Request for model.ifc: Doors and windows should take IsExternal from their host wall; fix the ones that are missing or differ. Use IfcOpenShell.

First a look at what the model holds.

```python
import ifcopenshell
import ifcopenshell.util.element

model = ifcopenshell.open("model.ifc")
print(model.schema)
seen = {}
for e in model.by_type("IfcDoor") + model.by_type("IfcWindow"):
    if not e.FillsVoids:
        continue
    host = e.FillsVoids[0].RelatingOpeningElement.VoidsElements[0].RelatingBuildingElement
    own = ifcopenshell.util.element.get_pset(e, f"Pset_{e.is_a()[3:].removesuffix('StandardCase')}Common", "IsExternal")
    wall = ifcopenshell.util.element.get_pset(host, "Pset_WallCommon", "IsExternal")
    seen[e.is_a(), own, wall] = seen.get((e.is_a(), own, wall), 0) + 1
for (cls, own, wall), count in sorted(seen.items(), key=str):
    print(count, cls, "IsExternal:", own, "| host wall:", wall)
```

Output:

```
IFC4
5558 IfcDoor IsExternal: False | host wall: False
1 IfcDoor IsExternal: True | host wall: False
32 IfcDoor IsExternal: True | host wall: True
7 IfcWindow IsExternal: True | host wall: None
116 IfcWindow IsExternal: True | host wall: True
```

```python
import ifcopenshell
import ifcopenshell.api.pset
import ifcopenshell.util.element

model = ifcopenshell.open("model.ifc")

count = 0
for ifc_class, pset_name in (("IfcDoor", "Pset_DoorCommon"), ("IfcWindow", "Pset_WindowCommon")):
    for e in model.by_type(ifc_class):
        if not e.FillsVoids:
            continue
        host = e.FillsVoids[0].RelatingOpeningElement.VoidsElements[0].RelatingBuildingElement
        external = ifcopenshell.util.element.get_pset(host, "Pset_WallCommon", "IsExternal")
        if external is None or ifcopenshell.util.element.get_pset(e, pset_name, "IsExternal") == external:
            continue
        pset = ifcopenshell.api.pset.add_pset(model, product=e, name=pset_name)
        ifcopenshell.api.pset.edit_pset(model, pset=pset, properties={"IsExternal": external})
        count += 1

print(count, "updated")

model.write("model-out.ifc")
```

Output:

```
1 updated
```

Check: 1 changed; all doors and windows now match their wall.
